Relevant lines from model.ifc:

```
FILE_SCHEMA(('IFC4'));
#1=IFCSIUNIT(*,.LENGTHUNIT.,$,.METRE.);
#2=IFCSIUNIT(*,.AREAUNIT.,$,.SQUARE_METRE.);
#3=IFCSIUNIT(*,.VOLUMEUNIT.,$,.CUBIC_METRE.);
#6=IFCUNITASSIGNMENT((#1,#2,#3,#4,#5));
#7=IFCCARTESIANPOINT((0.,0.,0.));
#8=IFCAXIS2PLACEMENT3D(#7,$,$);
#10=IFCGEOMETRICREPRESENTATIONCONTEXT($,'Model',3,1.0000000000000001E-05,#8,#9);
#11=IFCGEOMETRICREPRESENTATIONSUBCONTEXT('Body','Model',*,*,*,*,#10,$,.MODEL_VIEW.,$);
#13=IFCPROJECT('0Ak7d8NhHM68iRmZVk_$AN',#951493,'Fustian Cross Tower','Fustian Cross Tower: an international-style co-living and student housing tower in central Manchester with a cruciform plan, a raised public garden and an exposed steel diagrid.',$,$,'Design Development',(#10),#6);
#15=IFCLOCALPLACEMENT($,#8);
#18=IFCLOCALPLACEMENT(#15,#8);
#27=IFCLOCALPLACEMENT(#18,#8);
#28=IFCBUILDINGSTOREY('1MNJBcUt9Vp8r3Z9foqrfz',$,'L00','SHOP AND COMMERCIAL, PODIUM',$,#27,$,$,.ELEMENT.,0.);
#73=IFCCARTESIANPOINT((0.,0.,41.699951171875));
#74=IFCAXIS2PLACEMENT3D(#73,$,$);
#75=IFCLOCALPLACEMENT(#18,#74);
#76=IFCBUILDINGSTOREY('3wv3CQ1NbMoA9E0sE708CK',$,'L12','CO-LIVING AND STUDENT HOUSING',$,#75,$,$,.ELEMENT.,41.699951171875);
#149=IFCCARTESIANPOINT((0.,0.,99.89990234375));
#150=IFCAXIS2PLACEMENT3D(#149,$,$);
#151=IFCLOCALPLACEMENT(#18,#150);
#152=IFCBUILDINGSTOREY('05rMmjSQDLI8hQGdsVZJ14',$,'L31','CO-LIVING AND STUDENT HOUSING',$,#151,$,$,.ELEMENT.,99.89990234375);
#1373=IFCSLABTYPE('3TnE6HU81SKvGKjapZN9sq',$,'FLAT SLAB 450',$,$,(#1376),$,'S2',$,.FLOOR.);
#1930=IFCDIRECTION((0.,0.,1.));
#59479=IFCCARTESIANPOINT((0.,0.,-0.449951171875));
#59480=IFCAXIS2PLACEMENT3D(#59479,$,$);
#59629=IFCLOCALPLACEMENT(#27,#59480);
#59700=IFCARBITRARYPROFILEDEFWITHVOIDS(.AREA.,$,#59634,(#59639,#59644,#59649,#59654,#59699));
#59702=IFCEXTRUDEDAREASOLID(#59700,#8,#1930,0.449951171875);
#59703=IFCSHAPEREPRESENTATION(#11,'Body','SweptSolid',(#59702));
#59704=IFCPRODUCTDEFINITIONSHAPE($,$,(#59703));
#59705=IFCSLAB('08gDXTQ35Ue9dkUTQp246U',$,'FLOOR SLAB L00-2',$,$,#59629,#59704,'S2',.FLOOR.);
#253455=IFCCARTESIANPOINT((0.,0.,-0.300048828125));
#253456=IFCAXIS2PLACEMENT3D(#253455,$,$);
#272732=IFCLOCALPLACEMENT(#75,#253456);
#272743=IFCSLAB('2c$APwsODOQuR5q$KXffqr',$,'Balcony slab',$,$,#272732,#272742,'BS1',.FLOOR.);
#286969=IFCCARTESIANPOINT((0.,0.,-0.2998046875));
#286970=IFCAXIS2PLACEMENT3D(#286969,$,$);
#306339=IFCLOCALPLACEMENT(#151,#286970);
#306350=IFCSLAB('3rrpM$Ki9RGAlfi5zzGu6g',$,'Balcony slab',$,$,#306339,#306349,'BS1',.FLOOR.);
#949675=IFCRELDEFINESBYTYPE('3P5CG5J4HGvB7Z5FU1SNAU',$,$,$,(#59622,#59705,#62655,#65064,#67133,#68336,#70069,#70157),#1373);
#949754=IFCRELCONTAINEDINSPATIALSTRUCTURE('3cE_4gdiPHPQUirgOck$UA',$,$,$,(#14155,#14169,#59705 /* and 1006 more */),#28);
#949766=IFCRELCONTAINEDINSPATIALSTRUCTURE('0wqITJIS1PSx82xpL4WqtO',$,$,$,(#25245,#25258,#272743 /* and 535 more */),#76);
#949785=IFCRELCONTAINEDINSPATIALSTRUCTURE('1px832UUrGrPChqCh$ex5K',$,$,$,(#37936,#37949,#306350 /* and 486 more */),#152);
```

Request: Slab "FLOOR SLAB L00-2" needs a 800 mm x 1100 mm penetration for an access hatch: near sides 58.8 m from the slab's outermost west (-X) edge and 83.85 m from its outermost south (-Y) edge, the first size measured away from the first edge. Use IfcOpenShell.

```python
import numpy as np
import ifcopenshell
import ifcopenshell.api.feature
import ifcopenshell.api.geometry
import ifcopenshell.api.root
import ifcopenshell.geom
import ifcopenshell.util.placement
import ifcopenshell.util.representation
import ifcopenshell.util.shape
import ifcopenshell.util.unit

model = ifcopenshell.open("model.ifc")
unit_scale = ifcopenshell.util.unit.calculate_unit_scale(model)
settings = ifcopenshell.geom.settings()


def volume(element):
    """Net volume in cubic metres, openings subtracted."""
    shape = ifcopenshell.geom.create_shape(settings, element)
    return ifcopenshell.util.shape.get_volume(shape.geometry)


slab = model.by_guid("08gDXTQ35Ue9dkUTQp246U")
before = volume(slab)

# Extent in the slab's own axes, in metres. The edges named are its -X and -Y sides.
slab_shape = ifcopenshell.geom.create_shape(settings, slab)
vertices = ifcopenshell.util.shape.get_vertices(slab_shape.geometry)
x_min, y_min, bottom = vertices.min(axis=0)
top = vertices[:, 2].max()

opening = ifcopenshell.api.root.create_entity(model, ifc_class="IfcOpeningElement", name="Access hatch opening", predefined_type="OPENING")
context = ifcopenshell.util.representation.get_context(model, "Model", "Body", "MODEL_VIEW")
width, depth = 0.8, 1.1
outline = [(0.0, 0.0), (width, 0.0), (width, depth), (0.0, depth), (0.0, 0.0)]
# Overshoot both faces by 50 mm so the cut is clean.
shape = ifcopenshell.api.geometry.add_slab_representation(
    model, context=context, depth=top - bottom + 0.1, polyline=outline
)
ifcopenshell.api.geometry.assign_representation(model, product=opening, representation=shape)

matrix = ifcopenshell.util.placement.get_local_placement(slab.ObjectPlacement)
matrix[:, 3] = matrix @ np.append(np.array([x_min + 58.8, y_min + 83.85, bottom - 0.05]) / unit_scale, 1.0)
ifcopenshell.api.geometry.edit_object_placement(model, product=opening, matrix=matrix, is_si=False)
ifcopenshell.api.feature.add_feature(model, feature=opening, element=slab)

after = volume(slab)

print(f"slab volume {before:.3f} -> {after:.3f} m3")

model.write("model_updated.ifc")
```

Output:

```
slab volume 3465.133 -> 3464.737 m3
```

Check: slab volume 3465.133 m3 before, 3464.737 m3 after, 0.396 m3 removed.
